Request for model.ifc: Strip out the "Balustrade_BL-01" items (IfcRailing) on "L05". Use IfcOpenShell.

First a look at what the model holds.

```python
import ifcopenshell
import ifcopenshell.util.element

model = ifcopenshell.open("model.ifc")
print(model.schema)
storey = next(s for s in model.by_type("IfcBuildingStorey") if s.Name == "L05")
railings = [e for e in ifcopenshell.util.element.get_decomposition(storey) if e.is_a("IfcRailing")]
seen = {}
for e in railings:
    element_type = ifcopenshell.util.element.get_type(e)
    name = element_type.Name if element_type not in (None, e) else None
    seen[name] = seen.get(name, 0) + 1
for name, count in sorted(seen.items(), key=str):
    print(count, "x", name)
```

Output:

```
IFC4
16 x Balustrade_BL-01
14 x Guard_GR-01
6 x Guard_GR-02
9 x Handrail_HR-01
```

```python
import ifcopenshell
import ifcopenshell.api.root
import ifcopenshell.util.element

model = ifcopenshell.open("model.ifc")

storey = next(s for s in model.by_type("IfcBuildingStorey") if s.Name == "L05")
railings = [e for e in ifcopenshell.util.element.get_decomposition(storey) if e.is_a("IfcRailing")]
targets = [e for e in railings if (t := ifcopenshell.util.element.get_type(e)) not in (None, e) and t.Name == "Balustrade_BL-01"]

for e in targets:
    ifcopenshell.api.root.remove_product(model, product=e)
print(len(targets), "removed")

model.write("model-out.ifc")
```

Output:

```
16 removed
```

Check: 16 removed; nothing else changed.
